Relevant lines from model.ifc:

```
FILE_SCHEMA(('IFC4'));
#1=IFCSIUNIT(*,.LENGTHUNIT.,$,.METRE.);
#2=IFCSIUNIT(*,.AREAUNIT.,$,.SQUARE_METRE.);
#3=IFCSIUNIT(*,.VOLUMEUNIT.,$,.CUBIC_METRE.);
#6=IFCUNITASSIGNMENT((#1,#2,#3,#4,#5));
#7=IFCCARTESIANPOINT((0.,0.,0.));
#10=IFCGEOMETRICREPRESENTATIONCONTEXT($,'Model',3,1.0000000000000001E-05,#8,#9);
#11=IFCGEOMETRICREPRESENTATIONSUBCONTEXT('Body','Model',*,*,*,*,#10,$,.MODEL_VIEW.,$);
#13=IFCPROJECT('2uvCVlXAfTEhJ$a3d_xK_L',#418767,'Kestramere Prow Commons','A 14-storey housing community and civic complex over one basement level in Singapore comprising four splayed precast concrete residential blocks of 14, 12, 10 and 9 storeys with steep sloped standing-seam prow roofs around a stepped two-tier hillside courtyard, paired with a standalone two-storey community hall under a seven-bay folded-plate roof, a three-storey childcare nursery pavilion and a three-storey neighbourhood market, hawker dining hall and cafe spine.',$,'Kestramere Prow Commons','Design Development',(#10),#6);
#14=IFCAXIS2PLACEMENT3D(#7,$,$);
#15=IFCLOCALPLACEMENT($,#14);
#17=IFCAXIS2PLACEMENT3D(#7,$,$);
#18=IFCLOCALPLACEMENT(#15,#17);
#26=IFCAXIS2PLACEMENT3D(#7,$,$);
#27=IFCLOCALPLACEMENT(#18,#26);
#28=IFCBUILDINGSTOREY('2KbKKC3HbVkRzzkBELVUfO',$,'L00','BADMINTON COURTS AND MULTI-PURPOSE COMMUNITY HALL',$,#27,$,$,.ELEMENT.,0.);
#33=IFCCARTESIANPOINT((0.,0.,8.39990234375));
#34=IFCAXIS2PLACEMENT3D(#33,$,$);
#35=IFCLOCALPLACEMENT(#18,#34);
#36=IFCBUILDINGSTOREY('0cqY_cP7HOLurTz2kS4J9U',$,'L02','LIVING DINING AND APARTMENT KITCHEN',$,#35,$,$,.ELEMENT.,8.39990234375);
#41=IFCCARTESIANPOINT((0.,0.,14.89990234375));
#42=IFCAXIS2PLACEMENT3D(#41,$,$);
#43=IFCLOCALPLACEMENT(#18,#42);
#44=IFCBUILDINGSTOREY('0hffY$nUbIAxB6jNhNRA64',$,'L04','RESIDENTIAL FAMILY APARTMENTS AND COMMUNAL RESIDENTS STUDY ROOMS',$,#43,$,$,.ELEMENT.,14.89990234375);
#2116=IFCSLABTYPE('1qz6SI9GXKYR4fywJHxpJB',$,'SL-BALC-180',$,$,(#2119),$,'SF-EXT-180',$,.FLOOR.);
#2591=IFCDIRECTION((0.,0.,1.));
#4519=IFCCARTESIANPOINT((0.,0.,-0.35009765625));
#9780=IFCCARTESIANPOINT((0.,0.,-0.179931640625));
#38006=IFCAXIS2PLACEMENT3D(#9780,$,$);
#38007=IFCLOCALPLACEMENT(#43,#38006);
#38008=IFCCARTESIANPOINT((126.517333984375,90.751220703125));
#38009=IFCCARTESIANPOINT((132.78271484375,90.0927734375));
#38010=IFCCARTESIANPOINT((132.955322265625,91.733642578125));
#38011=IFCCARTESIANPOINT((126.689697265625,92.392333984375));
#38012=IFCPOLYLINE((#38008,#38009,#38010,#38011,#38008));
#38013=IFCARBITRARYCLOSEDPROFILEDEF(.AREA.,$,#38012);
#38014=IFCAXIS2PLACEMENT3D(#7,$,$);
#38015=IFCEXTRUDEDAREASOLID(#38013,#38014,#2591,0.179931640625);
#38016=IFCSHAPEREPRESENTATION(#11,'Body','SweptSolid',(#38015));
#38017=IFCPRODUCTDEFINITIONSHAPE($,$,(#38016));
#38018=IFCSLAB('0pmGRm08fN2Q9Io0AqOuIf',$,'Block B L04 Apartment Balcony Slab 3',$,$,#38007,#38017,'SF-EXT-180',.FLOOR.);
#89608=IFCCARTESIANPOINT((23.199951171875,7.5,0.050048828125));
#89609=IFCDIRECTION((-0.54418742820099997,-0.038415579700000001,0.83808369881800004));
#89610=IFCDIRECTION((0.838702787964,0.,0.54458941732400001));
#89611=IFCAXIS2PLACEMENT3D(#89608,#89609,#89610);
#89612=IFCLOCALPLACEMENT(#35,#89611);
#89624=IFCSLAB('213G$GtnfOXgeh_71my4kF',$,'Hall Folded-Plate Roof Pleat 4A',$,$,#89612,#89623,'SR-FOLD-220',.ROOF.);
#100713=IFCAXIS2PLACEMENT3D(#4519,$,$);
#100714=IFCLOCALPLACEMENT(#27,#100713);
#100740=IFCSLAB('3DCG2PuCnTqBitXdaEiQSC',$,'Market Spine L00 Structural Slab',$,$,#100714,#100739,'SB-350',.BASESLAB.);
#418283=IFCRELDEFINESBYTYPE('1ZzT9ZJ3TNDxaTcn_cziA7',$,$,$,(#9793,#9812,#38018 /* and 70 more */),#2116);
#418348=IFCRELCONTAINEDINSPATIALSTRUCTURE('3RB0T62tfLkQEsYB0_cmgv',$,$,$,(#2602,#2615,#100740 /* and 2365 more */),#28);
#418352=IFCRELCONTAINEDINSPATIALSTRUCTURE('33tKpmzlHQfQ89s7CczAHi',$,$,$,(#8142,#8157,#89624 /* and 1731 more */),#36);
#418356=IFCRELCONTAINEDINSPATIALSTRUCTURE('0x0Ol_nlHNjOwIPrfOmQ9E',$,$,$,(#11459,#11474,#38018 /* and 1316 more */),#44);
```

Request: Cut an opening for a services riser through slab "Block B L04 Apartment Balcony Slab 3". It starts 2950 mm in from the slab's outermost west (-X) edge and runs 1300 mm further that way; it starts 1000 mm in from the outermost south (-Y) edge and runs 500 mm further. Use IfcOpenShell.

```python
import numpy as np
import ifcopenshell
import ifcopenshell.api.feature
import ifcopenshell.api.geometry
import ifcopenshell.api.root
import ifcopenshell.geom
import ifcopenshell.util.placement
import ifcopenshell.util.representation
import ifcopenshell.util.shape
import ifcopenshell.util.unit

model = ifcopenshell.open("model.ifc")
unit_scale = ifcopenshell.util.unit.calculate_unit_scale(model)
settings = ifcopenshell.geom.settings()


def volume(element):
    """Net volume in cubic metres, openings subtracted."""
    shape = ifcopenshell.geom.create_shape(settings, element)
    return ifcopenshell.util.shape.get_volume(shape.geometry)


slab = model.by_guid("0pmGRm08fN2Q9Io0AqOuIf")
before = volume(slab)

# Extent in the slab's own axes, in metres. The edges named are its -X and -Y sides.
slab_shape = ifcopenshell.geom.create_shape(settings, slab)
vertices = ifcopenshell.util.shape.get_vertices(slab_shape.geometry)
x_min, y_min, bottom = vertices.min(axis=0)
top = vertices[:, 2].max()

opening = ifcopenshell.api.root.create_entity(model, ifc_class="IfcOpeningElement", name="Services riser opening", predefined_type="OPENING")
context = ifcopenshell.util.representation.get_context(model, "Model", "Body", "MODEL_VIEW")
width, depth = 1.3, 0.5
outline = [(0.0, 0.0), (width, 0.0), (width, depth), (0.0, depth), (0.0, 0.0)]
# Overshoot both faces by 50 mm so the cut is clean.
shape = ifcopenshell.api.geometry.add_slab_representation(
    model, context=context, depth=top - bottom + 0.1, polyline=outline
)
ifcopenshell.api.geometry.assign_representation(model, product=opening, representation=shape)

matrix = ifcopenshell.util.placement.get_local_placement(slab.ObjectPlacement)
matrix[:, 3] = matrix @ np.append(np.array([x_min + 2.95, y_min + 1, bottom - 0.05]) / unit_scale, 1.0)
ifcopenshell.api.geometry.edit_object_placement(model, product=opening, matrix=matrix, is_si=False)
ifcopenshell.api.feature.add_feature(model, feature=opening, element=slab)

after = volume(slab)

print(f"slab volume {before:.3f} -> {after:.3f} m3")

model.write("model_rev.ifc")
```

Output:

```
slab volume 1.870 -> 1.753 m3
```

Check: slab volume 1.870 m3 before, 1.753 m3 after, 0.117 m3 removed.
